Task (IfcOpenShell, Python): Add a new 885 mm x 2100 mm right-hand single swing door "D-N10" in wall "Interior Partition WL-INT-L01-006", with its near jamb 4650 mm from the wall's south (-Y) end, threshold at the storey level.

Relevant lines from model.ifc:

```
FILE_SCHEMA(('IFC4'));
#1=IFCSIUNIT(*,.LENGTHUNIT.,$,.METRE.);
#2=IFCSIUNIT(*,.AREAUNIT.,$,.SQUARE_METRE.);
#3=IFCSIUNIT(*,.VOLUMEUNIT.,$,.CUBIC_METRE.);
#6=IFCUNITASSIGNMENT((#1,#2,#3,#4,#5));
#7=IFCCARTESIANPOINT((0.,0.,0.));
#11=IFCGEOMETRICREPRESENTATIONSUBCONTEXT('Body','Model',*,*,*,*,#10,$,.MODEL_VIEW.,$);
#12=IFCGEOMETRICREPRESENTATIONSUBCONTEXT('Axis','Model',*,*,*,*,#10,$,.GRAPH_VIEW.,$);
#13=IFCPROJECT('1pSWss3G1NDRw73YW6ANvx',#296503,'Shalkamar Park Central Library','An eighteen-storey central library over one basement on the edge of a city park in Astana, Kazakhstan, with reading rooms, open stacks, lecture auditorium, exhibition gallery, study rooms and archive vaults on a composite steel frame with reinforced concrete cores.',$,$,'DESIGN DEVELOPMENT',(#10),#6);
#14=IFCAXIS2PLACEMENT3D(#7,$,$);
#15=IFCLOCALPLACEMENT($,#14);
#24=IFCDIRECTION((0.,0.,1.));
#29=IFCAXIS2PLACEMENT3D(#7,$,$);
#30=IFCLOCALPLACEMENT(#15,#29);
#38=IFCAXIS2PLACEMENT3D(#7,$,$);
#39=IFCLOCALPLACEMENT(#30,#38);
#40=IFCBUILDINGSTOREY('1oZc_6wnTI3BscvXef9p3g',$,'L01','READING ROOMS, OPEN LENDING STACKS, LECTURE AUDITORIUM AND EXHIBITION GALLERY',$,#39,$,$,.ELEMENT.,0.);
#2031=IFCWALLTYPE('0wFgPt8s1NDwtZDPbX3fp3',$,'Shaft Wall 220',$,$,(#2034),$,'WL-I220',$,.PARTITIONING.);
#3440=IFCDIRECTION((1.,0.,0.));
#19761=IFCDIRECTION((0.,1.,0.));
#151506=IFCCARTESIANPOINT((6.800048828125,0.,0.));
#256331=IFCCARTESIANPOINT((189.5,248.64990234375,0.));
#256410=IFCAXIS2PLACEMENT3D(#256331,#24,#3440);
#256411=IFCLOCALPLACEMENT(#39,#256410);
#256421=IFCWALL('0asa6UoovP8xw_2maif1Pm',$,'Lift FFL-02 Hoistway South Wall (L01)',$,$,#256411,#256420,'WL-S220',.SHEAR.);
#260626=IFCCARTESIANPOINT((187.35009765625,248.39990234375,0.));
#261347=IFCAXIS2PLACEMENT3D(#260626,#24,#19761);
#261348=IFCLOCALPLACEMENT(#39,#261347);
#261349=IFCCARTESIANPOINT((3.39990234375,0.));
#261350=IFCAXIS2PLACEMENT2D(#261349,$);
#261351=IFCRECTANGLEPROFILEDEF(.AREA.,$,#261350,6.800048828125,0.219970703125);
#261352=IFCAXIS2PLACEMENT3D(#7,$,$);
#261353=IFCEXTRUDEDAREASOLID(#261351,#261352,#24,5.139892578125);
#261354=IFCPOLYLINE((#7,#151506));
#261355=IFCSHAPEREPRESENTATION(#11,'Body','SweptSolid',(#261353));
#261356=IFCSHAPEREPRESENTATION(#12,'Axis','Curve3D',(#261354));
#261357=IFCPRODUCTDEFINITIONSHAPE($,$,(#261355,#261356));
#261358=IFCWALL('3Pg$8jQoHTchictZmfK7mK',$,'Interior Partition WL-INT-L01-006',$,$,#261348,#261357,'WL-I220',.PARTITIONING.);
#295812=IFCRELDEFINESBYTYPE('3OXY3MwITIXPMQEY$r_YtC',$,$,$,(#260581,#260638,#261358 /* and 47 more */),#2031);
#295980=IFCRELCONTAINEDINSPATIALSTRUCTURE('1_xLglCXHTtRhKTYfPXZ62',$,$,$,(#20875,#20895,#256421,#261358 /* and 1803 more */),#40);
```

```python
import numpy as np
import ifcopenshell
import ifcopenshell.api.feature
import ifcopenshell.api.geometry
import ifcopenshell.api.root
import ifcopenshell.api.spatial
import ifcopenshell.geom
import ifcopenshell.util.element
import ifcopenshell.util.placement
import ifcopenshell.util.representation
import ifcopenshell.util.shape
import ifcopenshell.util.unit

model = ifcopenshell.open("model.ifc")
unit_scale = ifcopenshell.util.unit.calculate_unit_scale(model)
settings = ifcopenshell.geom.settings()


def volume(element):
    """Net volume in cubic metres, openings subtracted."""
    shape = ifcopenshell.geom.create_shape(settings, element)
    return ifcopenshell.util.shape.get_volume(shape.geometry)


wall = model.by_guid("3Pg$8jQoHTchictZmfK7mK")
storey = ifcopenshell.util.element.get_container(wall, ifc_class="IfcBuildingStorey")
context = ifcopenshell.util.representation.get_context(model, "Model", "Body", "MODEL_VIEW")
before = volume(wall)

width, height, from_end, sill = 0.885, 2.1, 4.65, 0.0  # metres

# The wall runs along its own X axis, and the end named is its -X end.
wall_shape = ifcopenshell.geom.create_shape(settings, wall)
x, y, z = ifcopenshell.util.shape.get_vertices(wall_shape.geometry).T
start = x.min() + from_end
face, thickness = float(y.min()), float(y.max() - y.min())
wall_matrix = ifcopenshell.util.placement.get_local_placement(wall.ObjectPlacement)
level = ifcopenshell.util.placement.get_local_placement(storey.ObjectPlacement)[2, 3]


def in_wall(x, y):
    """Placement at x, y metres in the wall's axes, at sill height."""
    matrix = wall_matrix.copy()
    matrix[:, 3] = wall_matrix @ np.array([x / unit_scale, y / unit_scale, 0.0, 1.0])
    matrix[2, 3] = level + sill / unit_scale
    return matrix


# Opening: a box that overshoots both wall faces by 50 mm.
opening = ifcopenshell.api.root.create_entity(model, ifc_class="IfcOpeningElement", predefined_type="OPENING")
box = ifcopenshell.api.geometry.add_wall_representation(
    model, context=context, length=width, height=height, thickness=thickness + 0.1
)
ifcopenshell.api.geometry.assign_representation(model, product=opening, representation=box)
ifcopenshell.api.geometry.edit_object_placement(model, product=opening, matrix=in_wall(start, face - 0.05), is_si=False)
ifcopenshell.api.feature.add_feature(model, feature=opening, element=wall)

door = ifcopenshell.api.root.create_entity(model, ifc_class="IfcDoor", name="D-N10", predefined_type="DOOR")
door.OverallWidth, door.OverallHeight = width / unit_scale, height / unit_scale
door.OperationType = "SINGLE_SWING_RIGHT"
body = ifcopenshell.api.geometry.add_door_representation(
    model,
    context=context,
    overall_width=door.OverallWidth,
    overall_height=door.OverallHeight,
    operation_type="SINGLE_SWING_RIGHT",
    lining_properties={"LiningDepth": thickness / unit_scale, "ThresholdDepth": thickness / unit_scale},
)
ifcopenshell.api.geometry.assign_representation(model, product=door, representation=body)
ifcopenshell.api.spatial.assign_container(model, products=[door], relating_structure=storey)
ifcopenshell.api.feature.add_filling(model, opening=opening, element=door)

# The lining spans the wall, so the door starts at the wall face.
ifcopenshell.api.geometry.edit_object_placement(model, product=door, matrix=in_wall(start, face), is_si=False)

after = volume(wall)

print(f"wall volume {before:.3f} -> {after:.3f} m3")

model.write("model_updated.ifc")
```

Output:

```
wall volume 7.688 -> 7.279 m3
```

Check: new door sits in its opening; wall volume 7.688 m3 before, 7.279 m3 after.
